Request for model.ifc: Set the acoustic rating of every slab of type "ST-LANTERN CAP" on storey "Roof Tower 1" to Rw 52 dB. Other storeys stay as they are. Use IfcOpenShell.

First a look at what the model holds.

```python
import ifcopenshell
import ifcopenshell.util.element

model = ifcopenshell.open("model.ifc")
print(model.schema)
storey = next(s for s in model.by_type("IfcBuildingStorey") if s.Name == "Roof Tower 1")
slabs = [e for e in ifcopenshell.util.element.get_decomposition(storey) if e.is_a("IfcSlab")]
seen = {}
for e in slabs:
    element_type = ifcopenshell.util.element.get_type(e)
    key = (element_type.Name if element_type != e and element_type else None, ifcopenshell.util.element.get_pset(e, "Pset_SlabCommon", "AcousticRating"))
    seen[key] = seen.get(key, 0) + 1
for (name, value), count in sorted(seen.items(), key=str):
    print(count, "x", name, "|", value)
```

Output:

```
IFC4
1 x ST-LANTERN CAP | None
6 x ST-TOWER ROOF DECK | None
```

```python
import ifcopenshell
import ifcopenshell.api.pset
import ifcopenshell.util.element

model = ifcopenshell.open("model.ifc")

storey = next(s for s in model.by_type("IfcBuildingStorey") if s.Name == "Roof Tower 1")
slabs = [e for e in ifcopenshell.util.element.get_decomposition(storey) if e.is_a("IfcSlab")]

count = 0
for e in slabs:
    element_type = ifcopenshell.util.element.get_type(e)
    if element_type in (None, e) or element_type.Name != "ST-LANTERN CAP":
        continue
    # add_pset returns the element's existing set when there is one.
    pset = ifcopenshell.api.pset.add_pset(model, product=e, name="Pset_SlabCommon")
    ifcopenshell.api.pset.edit_pset(model, pset=pset, properties={"AcousticRating": "Rw 52 dB"})
    count += 1

print(count, "slabs updated")

model.write("model-out.ifc")
```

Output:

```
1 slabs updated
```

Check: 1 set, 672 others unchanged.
